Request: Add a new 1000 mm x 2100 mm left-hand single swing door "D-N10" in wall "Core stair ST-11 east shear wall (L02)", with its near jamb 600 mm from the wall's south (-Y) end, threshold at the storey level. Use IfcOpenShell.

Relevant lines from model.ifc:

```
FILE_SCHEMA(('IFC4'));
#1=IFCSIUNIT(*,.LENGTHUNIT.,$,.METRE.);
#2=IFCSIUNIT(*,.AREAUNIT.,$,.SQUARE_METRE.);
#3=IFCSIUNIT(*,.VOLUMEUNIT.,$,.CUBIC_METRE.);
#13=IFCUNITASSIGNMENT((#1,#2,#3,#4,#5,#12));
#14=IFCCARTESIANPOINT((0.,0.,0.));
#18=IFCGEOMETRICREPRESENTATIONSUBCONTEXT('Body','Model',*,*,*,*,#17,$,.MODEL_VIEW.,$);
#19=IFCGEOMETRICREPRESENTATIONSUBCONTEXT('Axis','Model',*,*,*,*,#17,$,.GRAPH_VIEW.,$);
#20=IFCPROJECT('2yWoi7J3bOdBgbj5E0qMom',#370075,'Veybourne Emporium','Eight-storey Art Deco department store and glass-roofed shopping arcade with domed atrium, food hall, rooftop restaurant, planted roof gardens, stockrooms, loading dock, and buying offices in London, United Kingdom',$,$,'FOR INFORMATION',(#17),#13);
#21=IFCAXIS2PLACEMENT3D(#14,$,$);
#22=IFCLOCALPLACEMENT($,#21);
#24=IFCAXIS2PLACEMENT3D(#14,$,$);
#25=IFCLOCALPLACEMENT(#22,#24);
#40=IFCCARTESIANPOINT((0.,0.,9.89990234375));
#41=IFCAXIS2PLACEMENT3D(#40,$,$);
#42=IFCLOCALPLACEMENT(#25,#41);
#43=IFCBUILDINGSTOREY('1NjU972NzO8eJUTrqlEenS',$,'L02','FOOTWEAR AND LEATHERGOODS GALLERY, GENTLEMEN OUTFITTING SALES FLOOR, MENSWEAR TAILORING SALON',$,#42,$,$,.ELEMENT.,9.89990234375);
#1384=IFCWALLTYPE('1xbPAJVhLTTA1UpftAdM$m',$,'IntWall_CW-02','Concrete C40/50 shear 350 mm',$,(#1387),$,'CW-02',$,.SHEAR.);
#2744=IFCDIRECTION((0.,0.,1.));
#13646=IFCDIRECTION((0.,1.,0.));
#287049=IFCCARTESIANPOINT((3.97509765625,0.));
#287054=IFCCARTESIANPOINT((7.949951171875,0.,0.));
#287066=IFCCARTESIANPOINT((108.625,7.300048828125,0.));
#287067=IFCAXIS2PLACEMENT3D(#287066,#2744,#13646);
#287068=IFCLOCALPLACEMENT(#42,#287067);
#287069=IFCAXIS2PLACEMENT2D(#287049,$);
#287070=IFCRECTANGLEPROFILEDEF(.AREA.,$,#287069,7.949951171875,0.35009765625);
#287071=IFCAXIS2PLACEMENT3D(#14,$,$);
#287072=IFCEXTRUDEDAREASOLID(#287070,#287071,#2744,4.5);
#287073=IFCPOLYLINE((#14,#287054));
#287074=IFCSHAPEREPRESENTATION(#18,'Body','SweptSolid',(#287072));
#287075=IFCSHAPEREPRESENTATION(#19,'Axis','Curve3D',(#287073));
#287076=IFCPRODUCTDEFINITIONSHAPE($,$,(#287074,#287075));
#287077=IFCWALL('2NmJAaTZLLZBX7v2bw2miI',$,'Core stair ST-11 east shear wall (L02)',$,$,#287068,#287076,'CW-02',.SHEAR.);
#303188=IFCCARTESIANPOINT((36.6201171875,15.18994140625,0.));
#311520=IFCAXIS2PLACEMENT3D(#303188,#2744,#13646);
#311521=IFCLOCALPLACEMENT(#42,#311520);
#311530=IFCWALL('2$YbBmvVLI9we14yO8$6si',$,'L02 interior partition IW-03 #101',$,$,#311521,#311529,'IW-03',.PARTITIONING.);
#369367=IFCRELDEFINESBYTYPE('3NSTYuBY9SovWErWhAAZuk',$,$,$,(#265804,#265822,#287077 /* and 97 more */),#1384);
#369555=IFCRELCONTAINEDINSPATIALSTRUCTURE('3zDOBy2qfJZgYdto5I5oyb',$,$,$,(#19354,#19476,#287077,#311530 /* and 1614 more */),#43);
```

```python
import numpy as np
import ifcopenshell
import ifcopenshell.api.feature
import ifcopenshell.api.geometry
import ifcopenshell.api.root
import ifcopenshell.api.spatial
import ifcopenshell.geom
import ifcopenshell.util.element
import ifcopenshell.util.placement
import ifcopenshell.util.representation
import ifcopenshell.util.shape
import ifcopenshell.util.unit

model = ifcopenshell.open("model.ifc")
unit_scale = ifcopenshell.util.unit.calculate_unit_scale(model)
settings = ifcopenshell.geom.settings()


def volume(element):
    """Net volume in cubic metres, openings subtracted."""
    shape = ifcopenshell.geom.create_shape(settings, element)
    return ifcopenshell.util.shape.get_volume(shape.geometry)


wall = model.by_guid("2NmJAaTZLLZBX7v2bw2miI")
storey = ifcopenshell.util.element.get_container(wall, ifc_class="IfcBuildingStorey")
context = ifcopenshell.util.representation.get_context(model, "Model", "Body", "MODEL_VIEW")
before = volume(wall)

width, height, from_end, sill = 1, 2.1, 0.6, 0.0  # metres

# The wall runs along its own X axis, and the end named is its -X end.
wall_shape = ifcopenshell.geom.create_shape(settings, wall)
x, y, z = ifcopenshell.util.shape.get_vertices(wall_shape.geometry).T
start = x.min() + from_end
face, thickness = float(y.min()), float(y.max() - y.min())
wall_matrix = ifcopenshell.util.placement.get_local_placement(wall.ObjectPlacement)
level = ifcopenshell.util.placement.get_local_placement(storey.ObjectPlacement)[2, 3]


def in_wall(x, y):
    """Placement at x, y metres in the wall's axes, at sill height."""
    matrix = wall_matrix.copy()
    matrix[:, 3] = wall_matrix @ np.array([x / unit_scale, y / unit_scale, 0.0, 1.0])
    matrix[2, 3] = level + sill / unit_scale
    return matrix


# Opening: a box that overshoots both wall faces by 50 mm.
opening = ifcopenshell.api.root.create_entity(model, ifc_class="IfcOpeningElement", predefined_type="OPENING")
box = ifcopenshell.api.geometry.add_wall_representation(
    model, context=context, length=width, height=height, thickness=thickness + 0.1
)
ifcopenshell.api.geometry.assign_representation(model, product=opening, representation=box)
ifcopenshell.api.geometry.edit_object_placement(model, product=opening, matrix=in_wall(start, face - 0.05), is_si=False)
ifcopenshell.api.feature.add_feature(model, feature=opening, element=wall)

door = ifcopenshell.api.root.create_entity(model, ifc_class="IfcDoor", name="D-N10", predefined_type="DOOR")
door.OverallWidth, door.OverallHeight = width / unit_scale, height / unit_scale
door.OperationType = "SINGLE_SWING_LEFT"
body = ifcopenshell.api.geometry.add_door_representation(
    model,
    context=context,
    overall_width=door.OverallWidth,
    overall_height=door.OverallHeight,
    operation_type="SINGLE_SWING_LEFT",
    lining_properties={"LiningDepth": thickness / unit_scale, "ThresholdDepth": thickness / unit_scale},
)
ifcopenshell.api.geometry.assign_representation(model, product=door, representation=body)
ifcopenshell.api.spatial.assign_container(model, products=[door], relating_structure=storey)
ifcopenshell.api.feature.add_filling(model, opening=opening, element=door)

# The lining spans the wall, so the door starts at the wall face.
ifcopenshell.api.geometry.edit_object_placement(model, product=door, matrix=in_wall(start, face), is_si=False)

after = volume(wall)

print(f"wall volume {before:.3f} -> {after:.3f} m3")

model.write("model_updated.ifc")
```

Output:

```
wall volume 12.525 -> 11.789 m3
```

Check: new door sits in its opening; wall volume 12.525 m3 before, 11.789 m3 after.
